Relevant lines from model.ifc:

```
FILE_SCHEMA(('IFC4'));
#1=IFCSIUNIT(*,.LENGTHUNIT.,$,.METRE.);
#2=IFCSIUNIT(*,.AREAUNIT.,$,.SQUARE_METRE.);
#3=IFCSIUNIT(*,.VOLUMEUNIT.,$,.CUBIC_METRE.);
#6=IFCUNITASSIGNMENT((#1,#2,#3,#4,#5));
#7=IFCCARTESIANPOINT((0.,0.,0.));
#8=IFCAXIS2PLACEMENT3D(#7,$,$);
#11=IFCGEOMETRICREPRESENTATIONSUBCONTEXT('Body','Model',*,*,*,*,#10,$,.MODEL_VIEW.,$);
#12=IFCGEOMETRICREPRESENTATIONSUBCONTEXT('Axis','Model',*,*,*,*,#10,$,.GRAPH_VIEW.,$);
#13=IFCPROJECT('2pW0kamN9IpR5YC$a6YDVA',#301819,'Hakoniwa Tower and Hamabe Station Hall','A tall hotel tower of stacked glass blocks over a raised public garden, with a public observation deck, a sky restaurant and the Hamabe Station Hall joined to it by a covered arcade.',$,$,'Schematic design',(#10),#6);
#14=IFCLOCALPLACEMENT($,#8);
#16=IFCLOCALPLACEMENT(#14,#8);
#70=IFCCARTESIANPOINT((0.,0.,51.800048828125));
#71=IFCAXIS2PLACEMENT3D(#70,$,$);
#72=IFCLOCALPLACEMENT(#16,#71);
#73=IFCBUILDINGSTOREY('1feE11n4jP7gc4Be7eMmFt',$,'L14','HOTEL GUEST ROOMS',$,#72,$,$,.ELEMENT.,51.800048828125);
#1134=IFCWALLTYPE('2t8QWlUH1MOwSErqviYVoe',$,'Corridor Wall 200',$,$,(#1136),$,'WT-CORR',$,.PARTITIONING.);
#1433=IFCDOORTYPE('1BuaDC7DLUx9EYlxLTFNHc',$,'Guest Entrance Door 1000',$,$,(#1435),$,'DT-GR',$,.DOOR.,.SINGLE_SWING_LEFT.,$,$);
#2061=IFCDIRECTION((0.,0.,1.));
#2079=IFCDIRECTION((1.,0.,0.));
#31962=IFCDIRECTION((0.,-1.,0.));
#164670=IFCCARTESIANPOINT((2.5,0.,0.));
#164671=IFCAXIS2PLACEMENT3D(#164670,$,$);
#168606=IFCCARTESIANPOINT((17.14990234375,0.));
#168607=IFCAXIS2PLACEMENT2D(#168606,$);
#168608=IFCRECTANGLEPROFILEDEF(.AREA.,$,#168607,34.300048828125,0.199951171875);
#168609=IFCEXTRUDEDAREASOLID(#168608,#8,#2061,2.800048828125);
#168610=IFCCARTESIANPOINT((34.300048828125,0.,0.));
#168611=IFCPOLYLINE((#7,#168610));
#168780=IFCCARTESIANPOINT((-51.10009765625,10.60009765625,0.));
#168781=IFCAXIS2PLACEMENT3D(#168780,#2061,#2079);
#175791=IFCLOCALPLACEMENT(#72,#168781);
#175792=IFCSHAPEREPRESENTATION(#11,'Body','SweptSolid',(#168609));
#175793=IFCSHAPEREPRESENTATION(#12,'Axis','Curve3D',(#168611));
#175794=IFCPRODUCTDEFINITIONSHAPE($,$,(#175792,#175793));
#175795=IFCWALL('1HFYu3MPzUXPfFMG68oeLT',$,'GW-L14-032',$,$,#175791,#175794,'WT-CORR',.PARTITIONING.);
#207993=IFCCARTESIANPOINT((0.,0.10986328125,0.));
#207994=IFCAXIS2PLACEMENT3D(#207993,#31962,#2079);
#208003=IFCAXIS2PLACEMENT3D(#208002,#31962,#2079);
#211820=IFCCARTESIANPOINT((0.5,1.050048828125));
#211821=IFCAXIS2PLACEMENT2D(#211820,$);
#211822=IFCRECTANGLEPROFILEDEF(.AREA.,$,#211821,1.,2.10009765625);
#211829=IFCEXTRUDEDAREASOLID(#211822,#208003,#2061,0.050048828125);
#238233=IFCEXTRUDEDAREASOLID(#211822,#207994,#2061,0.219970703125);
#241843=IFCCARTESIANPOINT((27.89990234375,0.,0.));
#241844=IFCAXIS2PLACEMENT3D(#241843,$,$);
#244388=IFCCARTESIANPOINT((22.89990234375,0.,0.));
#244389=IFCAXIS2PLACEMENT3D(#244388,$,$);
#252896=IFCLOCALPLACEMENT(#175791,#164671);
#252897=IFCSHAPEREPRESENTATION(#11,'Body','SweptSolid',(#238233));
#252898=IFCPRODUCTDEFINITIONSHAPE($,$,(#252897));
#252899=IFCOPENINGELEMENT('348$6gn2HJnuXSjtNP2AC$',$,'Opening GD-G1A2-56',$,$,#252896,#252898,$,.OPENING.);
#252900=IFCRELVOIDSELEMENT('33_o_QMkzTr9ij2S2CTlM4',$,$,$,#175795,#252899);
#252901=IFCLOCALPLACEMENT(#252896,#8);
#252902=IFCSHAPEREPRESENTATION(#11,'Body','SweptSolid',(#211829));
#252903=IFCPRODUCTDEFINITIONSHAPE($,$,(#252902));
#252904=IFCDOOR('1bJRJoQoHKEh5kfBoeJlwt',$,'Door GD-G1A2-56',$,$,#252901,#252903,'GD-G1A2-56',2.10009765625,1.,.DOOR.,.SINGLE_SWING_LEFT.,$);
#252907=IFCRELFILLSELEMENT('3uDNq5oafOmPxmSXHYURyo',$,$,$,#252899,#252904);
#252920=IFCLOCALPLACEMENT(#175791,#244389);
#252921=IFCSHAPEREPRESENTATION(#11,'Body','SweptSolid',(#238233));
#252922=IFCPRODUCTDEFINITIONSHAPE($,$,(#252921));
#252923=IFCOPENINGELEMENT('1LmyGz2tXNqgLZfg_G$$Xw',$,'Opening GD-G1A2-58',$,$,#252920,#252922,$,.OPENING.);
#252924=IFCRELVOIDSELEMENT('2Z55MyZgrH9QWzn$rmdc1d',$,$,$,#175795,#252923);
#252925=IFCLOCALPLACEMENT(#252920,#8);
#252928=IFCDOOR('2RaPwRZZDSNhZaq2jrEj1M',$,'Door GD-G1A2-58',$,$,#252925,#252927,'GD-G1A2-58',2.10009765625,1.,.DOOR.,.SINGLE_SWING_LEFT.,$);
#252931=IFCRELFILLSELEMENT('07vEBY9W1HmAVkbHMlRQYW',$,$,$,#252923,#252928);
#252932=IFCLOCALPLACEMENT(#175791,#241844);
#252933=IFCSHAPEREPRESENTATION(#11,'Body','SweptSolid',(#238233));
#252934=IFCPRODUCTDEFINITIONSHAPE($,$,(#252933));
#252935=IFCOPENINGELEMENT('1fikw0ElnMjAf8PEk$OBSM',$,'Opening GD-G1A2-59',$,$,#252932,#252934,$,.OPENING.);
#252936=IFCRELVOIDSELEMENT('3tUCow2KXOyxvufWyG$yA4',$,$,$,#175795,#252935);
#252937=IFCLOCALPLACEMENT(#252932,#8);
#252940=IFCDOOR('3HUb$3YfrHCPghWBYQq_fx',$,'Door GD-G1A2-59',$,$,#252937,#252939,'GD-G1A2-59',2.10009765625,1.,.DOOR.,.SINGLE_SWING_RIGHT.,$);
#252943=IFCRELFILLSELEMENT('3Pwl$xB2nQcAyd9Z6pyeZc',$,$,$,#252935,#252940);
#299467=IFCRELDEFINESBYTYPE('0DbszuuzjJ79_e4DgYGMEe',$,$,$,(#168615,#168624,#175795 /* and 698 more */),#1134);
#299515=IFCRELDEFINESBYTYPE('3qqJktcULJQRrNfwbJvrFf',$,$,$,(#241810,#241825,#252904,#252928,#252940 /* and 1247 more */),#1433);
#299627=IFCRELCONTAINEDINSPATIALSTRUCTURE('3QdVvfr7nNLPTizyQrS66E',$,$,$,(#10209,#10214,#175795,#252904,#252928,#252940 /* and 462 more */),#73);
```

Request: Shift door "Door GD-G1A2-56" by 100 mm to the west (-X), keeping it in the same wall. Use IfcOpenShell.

```python
import ifcopenshell
import ifcopenshell.api.geometry
import ifcopenshell.util.placement

model = ifcopenshell.open("model.ifc")

door = model.by_guid("1bJRJoQoHKEh5kfBoeJlwt")
opening = door.FillsVoids[0].RelatingOpeningElement
wall = opening.VoidsElements[0].RelatingBuildingElement

wall_matrix = ifcopenshell.util.placement.get_local_placement(wall.ObjectPlacement)
shift = wall_matrix[:3, 0] * -0.1
before = ifcopenshell.util.placement.get_local_placement(door.ObjectPlacement)[:3, 3].copy()

# The door is placed relative to its opening, so it follows when the opening moves.
matrix = ifcopenshell.util.placement.get_local_placement(opening.ObjectPlacement)
matrix[:3, 3] += shift
ifcopenshell.api.geometry.edit_object_placement(
    model, product=opening, matrix=matrix, is_si=False, should_transform_children=True
)

after = ifcopenshell.util.placement.get_local_placement(door.ObjectPlacement)[:3, 3]
print("door moved by", (after - before).round(3) + 0.0)

model.write("model_updated.ifc")
```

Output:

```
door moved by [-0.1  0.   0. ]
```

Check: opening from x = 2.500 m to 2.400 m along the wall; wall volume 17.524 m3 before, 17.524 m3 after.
